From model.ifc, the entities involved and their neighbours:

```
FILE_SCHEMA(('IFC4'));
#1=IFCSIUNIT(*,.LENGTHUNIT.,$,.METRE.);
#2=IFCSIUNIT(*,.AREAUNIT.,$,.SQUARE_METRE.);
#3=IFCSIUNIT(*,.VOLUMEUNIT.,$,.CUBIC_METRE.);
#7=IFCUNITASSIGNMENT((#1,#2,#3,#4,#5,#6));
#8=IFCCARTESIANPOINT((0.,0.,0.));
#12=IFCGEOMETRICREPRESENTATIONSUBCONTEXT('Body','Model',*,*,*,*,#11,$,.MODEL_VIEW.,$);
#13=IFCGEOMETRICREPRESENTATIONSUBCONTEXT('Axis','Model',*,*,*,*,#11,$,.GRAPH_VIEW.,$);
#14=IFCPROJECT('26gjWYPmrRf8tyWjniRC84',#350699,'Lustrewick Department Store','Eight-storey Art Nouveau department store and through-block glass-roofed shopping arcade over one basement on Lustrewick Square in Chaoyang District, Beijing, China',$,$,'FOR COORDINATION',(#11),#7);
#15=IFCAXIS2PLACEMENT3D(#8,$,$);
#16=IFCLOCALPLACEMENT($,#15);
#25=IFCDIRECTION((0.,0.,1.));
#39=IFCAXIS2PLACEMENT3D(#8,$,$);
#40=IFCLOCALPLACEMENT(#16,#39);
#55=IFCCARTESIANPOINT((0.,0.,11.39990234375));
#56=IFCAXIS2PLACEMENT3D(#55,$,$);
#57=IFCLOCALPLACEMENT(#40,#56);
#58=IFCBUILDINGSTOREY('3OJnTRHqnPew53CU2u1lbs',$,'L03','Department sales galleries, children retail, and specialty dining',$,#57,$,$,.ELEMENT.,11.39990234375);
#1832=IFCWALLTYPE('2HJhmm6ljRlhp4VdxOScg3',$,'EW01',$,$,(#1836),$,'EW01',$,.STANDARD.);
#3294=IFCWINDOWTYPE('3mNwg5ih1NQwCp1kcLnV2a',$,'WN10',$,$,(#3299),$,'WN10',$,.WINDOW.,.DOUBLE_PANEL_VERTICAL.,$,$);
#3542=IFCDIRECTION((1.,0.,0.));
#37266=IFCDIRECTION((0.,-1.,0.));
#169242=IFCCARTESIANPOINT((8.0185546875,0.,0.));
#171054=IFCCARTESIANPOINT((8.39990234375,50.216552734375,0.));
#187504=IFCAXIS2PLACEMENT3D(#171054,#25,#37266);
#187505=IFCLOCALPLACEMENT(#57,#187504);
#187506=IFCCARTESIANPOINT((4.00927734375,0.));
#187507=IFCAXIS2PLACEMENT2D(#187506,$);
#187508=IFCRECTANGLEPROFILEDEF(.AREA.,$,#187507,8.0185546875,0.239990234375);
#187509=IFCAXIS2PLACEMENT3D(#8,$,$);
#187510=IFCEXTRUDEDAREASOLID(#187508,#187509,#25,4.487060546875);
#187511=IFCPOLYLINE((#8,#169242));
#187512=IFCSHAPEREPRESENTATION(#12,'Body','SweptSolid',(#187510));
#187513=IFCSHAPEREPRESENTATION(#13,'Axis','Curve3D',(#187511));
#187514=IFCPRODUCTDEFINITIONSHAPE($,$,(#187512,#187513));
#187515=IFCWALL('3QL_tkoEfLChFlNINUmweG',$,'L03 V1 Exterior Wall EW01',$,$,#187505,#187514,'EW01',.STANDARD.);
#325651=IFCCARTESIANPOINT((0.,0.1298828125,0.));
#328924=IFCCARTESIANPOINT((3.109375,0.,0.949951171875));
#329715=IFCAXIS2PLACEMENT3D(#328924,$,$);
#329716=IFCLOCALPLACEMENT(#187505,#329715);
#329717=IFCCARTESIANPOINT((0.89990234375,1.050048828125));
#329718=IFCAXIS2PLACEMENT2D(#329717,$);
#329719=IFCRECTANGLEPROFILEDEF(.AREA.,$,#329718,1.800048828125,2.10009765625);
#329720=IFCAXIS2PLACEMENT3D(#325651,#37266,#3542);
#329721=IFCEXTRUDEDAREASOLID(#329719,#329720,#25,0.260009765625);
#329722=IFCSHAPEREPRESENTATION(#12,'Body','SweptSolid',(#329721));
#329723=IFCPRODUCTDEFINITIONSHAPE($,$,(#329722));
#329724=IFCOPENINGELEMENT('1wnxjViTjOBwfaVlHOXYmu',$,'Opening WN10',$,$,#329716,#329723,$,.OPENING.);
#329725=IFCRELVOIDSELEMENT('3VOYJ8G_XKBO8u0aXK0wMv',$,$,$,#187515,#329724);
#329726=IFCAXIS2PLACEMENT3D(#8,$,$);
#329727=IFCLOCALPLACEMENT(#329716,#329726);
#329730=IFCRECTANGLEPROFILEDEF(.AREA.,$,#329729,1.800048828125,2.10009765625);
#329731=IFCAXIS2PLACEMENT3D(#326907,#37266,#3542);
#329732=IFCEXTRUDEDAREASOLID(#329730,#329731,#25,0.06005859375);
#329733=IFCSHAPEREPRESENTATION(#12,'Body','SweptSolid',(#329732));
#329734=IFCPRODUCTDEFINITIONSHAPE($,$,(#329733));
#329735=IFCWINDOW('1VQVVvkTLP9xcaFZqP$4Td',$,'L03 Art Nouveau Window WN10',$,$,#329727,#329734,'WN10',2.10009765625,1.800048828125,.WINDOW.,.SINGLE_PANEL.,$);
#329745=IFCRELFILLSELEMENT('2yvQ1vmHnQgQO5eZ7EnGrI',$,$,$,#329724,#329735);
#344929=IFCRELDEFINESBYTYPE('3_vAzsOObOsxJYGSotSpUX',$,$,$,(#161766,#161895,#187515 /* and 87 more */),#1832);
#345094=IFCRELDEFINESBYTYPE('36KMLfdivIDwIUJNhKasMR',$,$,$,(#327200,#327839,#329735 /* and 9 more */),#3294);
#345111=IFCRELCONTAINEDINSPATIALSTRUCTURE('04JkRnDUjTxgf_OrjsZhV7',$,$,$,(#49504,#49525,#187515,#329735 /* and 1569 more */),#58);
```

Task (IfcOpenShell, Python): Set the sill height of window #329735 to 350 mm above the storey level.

```python
import numpy as np
import ifcopenshell
import ifcopenshell.api.geometry
import ifcopenshell.geom
import ifcopenshell.util.element
import ifcopenshell.util.placement
import ifcopenshell.util.shape
import ifcopenshell.util.unit

model = ifcopenshell.open("model.ifc")
unit_scale = ifcopenshell.util.unit.calculate_unit_scale(model)

window = model.by_id(329735)
opening = window.FillsVoids[0].RelatingOpeningElement
storey = ifcopenshell.util.element.get_container(window, ifc_class="IfcBuildingStorey")
level = ifcopenshell.util.placement.get_local_placement(storey.ObjectPlacement)[2, 3]

# The opening's origin need not be at the sill, so measure its lowest point.
shape = ifcopenshell.geom.create_shape(ifcopenshell.geom.settings(), opening)
bottom = ifcopenshell.util.shape.get_shape_bottom_elevation(shape, shape.geometry) / unit_scale
dz = level + 0.35 - bottom

shift = np.array([0.0, 0.0, dz])
# The window is placed relative to its opening, so it follows when the opening moves.
matrix = ifcopenshell.util.placement.get_local_placement(opening.ObjectPlacement)
matrix[:3, 3] += shift
ifcopenshell.api.geometry.edit_object_placement(
    model, product=opening, matrix=matrix, is_si=False, should_transform_children=True
)

print(f"moved by {dz * unit_scale:+.3f} m")

model.write("model_rev.ifc")
```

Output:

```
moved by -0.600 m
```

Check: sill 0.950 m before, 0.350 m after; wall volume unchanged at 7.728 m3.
